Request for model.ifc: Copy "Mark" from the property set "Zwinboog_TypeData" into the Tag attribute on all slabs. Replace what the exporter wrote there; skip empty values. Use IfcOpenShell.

First a look at what the model holds.

```python
import ifcopenshell
import ifcopenshell.util.element

model = ifcopenshell.open("model.ifc")
print(model.schema)
slabs = model.by_type("IfcSlab")
print(len(slabs), "slabs")
for e in slabs[:8]:
    source = ifcopenshell.util.element.get_pset(e, "Zwinboog_TypeData", "Mark")
    target = e.Tag
    print(e.id(), repr(source), repr(target), sep=" | ")
```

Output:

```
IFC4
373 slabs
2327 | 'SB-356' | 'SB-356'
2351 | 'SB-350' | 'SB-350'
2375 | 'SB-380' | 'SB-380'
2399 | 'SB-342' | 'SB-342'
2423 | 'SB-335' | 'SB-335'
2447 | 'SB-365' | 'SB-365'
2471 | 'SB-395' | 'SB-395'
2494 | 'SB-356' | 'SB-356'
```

```python
import ifcopenshell
import ifcopenshell.util.element

model = ifcopenshell.open("model.ifc")

count = 0
for e in model.by_type("IfcSlab"):
    value = ifcopenshell.util.element.get_pset(e, "Zwinboog_TypeData", "Mark")
    current = e.Tag
    if not value or not value.strip() or current == value:
        continue
    e.Tag = value
    count += 1

print(count, "slabs updated")

model.write("model-out.ifc")
```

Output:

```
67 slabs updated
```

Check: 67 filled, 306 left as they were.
